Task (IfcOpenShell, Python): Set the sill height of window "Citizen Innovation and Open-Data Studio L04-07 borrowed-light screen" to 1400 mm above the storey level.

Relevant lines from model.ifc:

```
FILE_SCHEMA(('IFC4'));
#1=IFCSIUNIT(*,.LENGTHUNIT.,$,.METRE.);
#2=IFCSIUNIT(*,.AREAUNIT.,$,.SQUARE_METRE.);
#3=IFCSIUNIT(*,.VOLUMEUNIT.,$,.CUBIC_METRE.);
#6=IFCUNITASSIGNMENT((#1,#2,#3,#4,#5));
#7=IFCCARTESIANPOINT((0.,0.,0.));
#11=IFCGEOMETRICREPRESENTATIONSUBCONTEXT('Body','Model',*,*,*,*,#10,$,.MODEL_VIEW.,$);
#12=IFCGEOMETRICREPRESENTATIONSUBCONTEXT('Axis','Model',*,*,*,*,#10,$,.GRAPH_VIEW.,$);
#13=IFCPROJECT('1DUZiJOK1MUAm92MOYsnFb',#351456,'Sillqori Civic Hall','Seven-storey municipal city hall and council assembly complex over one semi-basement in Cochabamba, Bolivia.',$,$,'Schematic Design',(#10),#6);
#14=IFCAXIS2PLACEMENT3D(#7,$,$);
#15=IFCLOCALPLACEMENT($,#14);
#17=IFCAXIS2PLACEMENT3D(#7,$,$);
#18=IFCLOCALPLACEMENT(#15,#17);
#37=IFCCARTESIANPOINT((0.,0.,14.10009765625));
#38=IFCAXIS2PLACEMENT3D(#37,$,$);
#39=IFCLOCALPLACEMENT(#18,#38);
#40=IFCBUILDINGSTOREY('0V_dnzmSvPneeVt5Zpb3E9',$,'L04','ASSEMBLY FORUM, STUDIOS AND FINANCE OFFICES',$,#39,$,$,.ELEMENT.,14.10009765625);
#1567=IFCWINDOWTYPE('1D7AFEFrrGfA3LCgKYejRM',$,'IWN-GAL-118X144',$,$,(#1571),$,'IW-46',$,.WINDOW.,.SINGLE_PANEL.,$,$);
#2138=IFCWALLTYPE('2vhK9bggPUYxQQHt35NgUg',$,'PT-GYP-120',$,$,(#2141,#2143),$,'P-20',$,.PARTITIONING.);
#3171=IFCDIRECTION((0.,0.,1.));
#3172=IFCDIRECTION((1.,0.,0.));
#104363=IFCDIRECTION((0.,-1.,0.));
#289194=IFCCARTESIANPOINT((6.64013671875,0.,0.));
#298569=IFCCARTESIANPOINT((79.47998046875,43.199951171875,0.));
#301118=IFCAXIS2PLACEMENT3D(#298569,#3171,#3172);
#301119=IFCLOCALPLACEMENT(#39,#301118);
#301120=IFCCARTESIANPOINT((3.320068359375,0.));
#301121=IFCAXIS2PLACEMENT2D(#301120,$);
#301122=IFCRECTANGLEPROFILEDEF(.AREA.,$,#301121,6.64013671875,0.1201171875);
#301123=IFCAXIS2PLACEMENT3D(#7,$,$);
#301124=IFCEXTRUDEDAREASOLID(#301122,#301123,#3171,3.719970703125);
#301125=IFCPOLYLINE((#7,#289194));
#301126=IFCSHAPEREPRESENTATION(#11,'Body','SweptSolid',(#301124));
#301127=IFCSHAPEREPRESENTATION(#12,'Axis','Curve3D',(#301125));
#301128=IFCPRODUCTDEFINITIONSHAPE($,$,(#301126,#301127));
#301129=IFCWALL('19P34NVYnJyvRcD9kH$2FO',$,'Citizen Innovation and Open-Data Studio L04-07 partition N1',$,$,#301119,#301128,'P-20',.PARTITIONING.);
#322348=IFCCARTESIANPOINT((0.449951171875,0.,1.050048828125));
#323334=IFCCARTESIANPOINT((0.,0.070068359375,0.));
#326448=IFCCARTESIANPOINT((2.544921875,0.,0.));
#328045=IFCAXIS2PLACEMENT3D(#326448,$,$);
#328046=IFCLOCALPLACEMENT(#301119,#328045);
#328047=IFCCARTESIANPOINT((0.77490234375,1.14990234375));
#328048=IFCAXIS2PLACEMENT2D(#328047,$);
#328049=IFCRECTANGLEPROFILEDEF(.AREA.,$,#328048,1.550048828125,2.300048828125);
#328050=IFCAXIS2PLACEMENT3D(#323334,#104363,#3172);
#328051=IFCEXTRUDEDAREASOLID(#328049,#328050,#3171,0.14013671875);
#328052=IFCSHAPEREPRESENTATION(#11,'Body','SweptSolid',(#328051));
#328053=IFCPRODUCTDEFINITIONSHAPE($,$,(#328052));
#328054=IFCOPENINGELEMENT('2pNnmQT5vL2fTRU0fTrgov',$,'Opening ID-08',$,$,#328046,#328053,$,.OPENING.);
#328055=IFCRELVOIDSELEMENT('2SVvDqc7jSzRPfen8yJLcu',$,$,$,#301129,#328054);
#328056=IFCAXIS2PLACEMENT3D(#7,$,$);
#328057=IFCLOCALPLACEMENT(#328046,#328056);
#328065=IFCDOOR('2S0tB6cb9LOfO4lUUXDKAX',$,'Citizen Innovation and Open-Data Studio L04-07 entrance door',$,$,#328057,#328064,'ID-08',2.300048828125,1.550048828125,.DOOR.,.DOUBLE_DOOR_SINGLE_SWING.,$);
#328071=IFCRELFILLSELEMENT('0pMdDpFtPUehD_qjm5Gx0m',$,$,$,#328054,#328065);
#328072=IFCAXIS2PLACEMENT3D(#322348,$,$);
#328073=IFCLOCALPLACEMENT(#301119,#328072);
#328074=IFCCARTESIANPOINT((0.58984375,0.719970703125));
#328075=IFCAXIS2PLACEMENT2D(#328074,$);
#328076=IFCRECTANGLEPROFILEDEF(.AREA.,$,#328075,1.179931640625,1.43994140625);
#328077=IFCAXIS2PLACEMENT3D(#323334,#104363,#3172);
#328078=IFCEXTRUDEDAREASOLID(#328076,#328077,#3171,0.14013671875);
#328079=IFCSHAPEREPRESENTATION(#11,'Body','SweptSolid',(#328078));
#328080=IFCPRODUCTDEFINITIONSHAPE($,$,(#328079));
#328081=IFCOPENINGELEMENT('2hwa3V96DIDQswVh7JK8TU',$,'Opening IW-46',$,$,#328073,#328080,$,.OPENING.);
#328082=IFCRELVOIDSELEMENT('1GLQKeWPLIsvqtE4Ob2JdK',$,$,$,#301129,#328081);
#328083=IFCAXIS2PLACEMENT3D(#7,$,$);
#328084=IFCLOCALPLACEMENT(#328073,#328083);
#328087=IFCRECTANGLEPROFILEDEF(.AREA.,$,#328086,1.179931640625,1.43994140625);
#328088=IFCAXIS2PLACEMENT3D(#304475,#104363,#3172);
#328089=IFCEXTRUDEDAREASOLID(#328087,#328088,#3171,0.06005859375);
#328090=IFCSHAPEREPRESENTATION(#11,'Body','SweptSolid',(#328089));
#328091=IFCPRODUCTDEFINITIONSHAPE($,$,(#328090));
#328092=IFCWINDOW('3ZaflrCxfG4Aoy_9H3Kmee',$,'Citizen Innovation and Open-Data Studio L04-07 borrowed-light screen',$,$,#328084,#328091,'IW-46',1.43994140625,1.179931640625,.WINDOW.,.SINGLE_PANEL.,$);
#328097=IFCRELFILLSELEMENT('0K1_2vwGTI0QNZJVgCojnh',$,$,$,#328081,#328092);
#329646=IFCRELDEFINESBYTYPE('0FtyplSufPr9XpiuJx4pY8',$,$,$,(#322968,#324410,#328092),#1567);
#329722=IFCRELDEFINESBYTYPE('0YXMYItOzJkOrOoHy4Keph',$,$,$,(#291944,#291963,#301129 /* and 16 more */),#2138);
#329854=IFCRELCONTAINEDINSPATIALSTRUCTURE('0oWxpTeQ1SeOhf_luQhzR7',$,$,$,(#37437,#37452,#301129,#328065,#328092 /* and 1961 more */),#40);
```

```python
import numpy as np
import ifcopenshell
import ifcopenshell.api.geometry
import ifcopenshell.geom
import ifcopenshell.util.element
import ifcopenshell.util.placement
import ifcopenshell.util.shape
import ifcopenshell.util.unit

model = ifcopenshell.open("model.ifc")
unit_scale = ifcopenshell.util.unit.calculate_unit_scale(model)

window = model.by_guid("3ZaflrCxfG4Aoy_9H3Kmee")
opening = window.FillsVoids[0].RelatingOpeningElement
storey = ifcopenshell.util.element.get_container(window, ifc_class="IfcBuildingStorey")
level = ifcopenshell.util.placement.get_local_placement(storey.ObjectPlacement)[2, 3]

# The opening's origin need not be at the sill, so measure its lowest point.
shape = ifcopenshell.geom.create_shape(ifcopenshell.geom.settings(), opening)
bottom = ifcopenshell.util.shape.get_shape_bottom_elevation(shape, shape.geometry) / unit_scale
dz = level + 1.4 - bottom

shift = np.array([0.0, 0.0, dz])
# The window is placed relative to its opening, so it follows when the opening moves.
matrix = ifcopenshell.util.placement.get_local_placement(opening.ObjectPlacement)
matrix[:3, 3] += shift
ifcopenshell.api.geometry.edit_object_placement(
    model, product=opening, matrix=matrix, is_si=False, should_transform_children=True
)

print(f"moved by {dz * unit_scale:+.3f} m")

model.write("model_v2.ifc")
```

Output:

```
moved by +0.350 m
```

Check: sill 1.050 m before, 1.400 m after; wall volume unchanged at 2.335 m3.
